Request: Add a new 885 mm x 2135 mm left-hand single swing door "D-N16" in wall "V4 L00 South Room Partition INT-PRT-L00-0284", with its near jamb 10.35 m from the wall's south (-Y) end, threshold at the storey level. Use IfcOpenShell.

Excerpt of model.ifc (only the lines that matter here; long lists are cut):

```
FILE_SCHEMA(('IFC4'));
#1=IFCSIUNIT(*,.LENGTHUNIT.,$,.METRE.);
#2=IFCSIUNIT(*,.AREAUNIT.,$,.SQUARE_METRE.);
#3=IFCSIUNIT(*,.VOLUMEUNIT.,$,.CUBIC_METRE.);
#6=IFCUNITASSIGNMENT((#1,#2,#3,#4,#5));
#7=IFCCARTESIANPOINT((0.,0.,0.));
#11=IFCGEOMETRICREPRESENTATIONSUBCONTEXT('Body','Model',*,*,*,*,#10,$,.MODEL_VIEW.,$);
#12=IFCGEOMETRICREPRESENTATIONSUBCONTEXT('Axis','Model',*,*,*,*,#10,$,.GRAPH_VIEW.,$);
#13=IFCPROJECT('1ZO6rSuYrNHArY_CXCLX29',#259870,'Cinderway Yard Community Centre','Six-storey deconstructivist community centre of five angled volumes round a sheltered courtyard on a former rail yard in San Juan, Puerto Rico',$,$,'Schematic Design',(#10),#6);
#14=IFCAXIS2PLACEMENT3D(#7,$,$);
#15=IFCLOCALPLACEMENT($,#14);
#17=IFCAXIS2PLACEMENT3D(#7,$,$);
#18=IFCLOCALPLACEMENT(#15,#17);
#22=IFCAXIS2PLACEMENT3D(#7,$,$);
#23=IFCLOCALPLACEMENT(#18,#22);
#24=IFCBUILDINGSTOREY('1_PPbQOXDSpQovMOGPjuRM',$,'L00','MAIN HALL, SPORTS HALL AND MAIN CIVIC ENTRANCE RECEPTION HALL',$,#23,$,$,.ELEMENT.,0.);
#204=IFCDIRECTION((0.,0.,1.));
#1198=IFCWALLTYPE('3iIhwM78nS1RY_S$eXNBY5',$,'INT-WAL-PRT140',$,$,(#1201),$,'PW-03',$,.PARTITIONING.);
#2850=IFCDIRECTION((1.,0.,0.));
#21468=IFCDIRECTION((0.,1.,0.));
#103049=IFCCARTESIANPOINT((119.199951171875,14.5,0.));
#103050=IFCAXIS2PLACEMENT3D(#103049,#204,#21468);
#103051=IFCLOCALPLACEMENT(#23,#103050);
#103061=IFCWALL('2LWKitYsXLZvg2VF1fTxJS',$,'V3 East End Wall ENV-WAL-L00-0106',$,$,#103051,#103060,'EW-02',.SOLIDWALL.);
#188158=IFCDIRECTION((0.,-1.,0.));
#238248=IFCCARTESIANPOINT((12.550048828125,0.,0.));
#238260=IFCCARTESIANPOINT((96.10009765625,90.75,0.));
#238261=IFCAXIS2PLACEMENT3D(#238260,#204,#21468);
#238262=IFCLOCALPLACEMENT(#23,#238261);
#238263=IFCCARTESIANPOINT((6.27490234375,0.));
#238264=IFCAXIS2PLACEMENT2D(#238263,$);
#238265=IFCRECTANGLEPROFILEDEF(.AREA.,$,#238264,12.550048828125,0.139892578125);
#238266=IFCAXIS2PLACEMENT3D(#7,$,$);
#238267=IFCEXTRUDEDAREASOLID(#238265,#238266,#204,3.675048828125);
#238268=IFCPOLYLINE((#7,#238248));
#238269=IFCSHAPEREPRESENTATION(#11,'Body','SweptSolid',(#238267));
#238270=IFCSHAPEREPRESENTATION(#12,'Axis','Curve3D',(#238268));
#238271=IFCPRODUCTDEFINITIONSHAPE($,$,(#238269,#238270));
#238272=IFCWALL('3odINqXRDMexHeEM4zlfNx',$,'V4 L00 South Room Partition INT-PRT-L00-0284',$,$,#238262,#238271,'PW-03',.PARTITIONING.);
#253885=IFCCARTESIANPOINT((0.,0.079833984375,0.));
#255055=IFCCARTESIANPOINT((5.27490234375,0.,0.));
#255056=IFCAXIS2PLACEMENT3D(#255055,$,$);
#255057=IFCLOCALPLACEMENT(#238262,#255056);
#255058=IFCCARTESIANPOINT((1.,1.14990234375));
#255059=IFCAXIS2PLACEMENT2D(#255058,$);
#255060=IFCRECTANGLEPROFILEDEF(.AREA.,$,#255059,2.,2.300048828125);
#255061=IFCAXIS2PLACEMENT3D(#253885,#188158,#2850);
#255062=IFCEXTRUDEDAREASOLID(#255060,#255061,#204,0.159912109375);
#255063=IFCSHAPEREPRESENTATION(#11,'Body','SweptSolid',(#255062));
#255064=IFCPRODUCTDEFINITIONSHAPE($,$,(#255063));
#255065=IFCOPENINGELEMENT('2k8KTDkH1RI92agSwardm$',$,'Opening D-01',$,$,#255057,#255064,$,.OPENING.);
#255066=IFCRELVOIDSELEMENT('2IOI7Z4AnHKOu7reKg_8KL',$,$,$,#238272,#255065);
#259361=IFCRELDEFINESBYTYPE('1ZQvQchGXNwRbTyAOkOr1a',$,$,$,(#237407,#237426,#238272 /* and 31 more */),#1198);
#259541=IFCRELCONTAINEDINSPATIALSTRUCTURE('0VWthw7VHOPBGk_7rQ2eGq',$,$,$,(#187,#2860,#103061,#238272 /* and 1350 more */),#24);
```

```python
import numpy as np
import ifcopenshell
import ifcopenshell.api.feature
import ifcopenshell.api.geometry
import ifcopenshell.api.root
import ifcopenshell.api.spatial
import ifcopenshell.geom
import ifcopenshell.util.element
import ifcopenshell.util.placement
import ifcopenshell.util.representation
import ifcopenshell.util.shape
import ifcopenshell.util.unit

model = ifcopenshell.open("model.ifc")
unit_scale = ifcopenshell.util.unit.calculate_unit_scale(model)
settings = ifcopenshell.geom.settings()


def volume(element):
    """Net volume in cubic metres, openings subtracted."""
    shape = ifcopenshell.geom.create_shape(settings, element)
    return ifcopenshell.util.shape.get_volume(shape.geometry)


wall = model.by_guid("3odINqXRDMexHeEM4zlfNx")
storey = ifcopenshell.util.element.get_container(wall, ifc_class="IfcBuildingStorey")
context = ifcopenshell.util.representation.get_context(model, "Model", "Body", "MODEL_VIEW")
before = volume(wall)

width, height, from_end, sill = 0.885, 2.135, 10.35, 0.0  # metres

# The wall runs along its own X axis, and the end named is its -X end.
wall_shape = ifcopenshell.geom.create_shape(settings, wall)
x, y, z = ifcopenshell.util.shape.get_vertices(wall_shape.geometry).T
start = x.min() + from_end
face, thickness = float(y.min()), float(y.max() - y.min())
wall_matrix = ifcopenshell.util.placement.get_local_placement(wall.ObjectPlacement)
level = ifcopenshell.util.placement.get_local_placement(storey.ObjectPlacement)[2, 3]


def in_wall(x, y):
    """Placement at x, y metres in the wall's axes, at sill height."""
    matrix = wall_matrix.copy()
    matrix[:, 3] = wall_matrix @ np.array([x / unit_scale, y / unit_scale, 0.0, 1.0])
    matrix[2, 3] = level + sill / unit_scale
    return matrix


# Opening: a box that overshoots both wall faces by 50 mm.
opening = ifcopenshell.api.root.create_entity(model, ifc_class="IfcOpeningElement", predefined_type="OPENING")
box = ifcopenshell.api.geometry.add_wall_representation(
    model, context=context, length=width, height=height, thickness=thickness + 0.1
)
ifcopenshell.api.geometry.assign_representation(model, product=opening, representation=box)
ifcopenshell.api.geometry.edit_object_placement(model, product=opening, matrix=in_wall(start, face - 0.05), is_si=False)
ifcopenshell.api.feature.add_feature(model, feature=opening, element=wall)

door = ifcopenshell.api.root.create_entity(model, ifc_class="IfcDoor", name="D-N16", predefined_type="DOOR")
door.OverallWidth, door.OverallHeight = width / unit_scale, height / unit_scale
door.OperationType = "SINGLE_SWING_LEFT"
body = ifcopenshell.api.geometry.add_door_representation(
    model,
    context=context,
    overall_width=door.OverallWidth,
    overall_height=door.OverallHeight,
    operation_type="SINGLE_SWING_LEFT",
    lining_properties={"LiningDepth": thickness / unit_scale, "ThresholdDepth": thickness / unit_scale},
)
ifcopenshell.api.geometry.assign_representation(model, product=door, representation=body)
ifcopenshell.api.spatial.assign_container(model, products=[door], relating_structure=storey)
ifcopenshell.api.feature.add_filling(model, opening=opening, element=door)

# The lining spans the wall, so the door starts at the wall face.
ifcopenshell.api.geometry.edit_object_placement(model, product=door, matrix=in_wall(start, face), is_si=False)

after = volume(wall)

print(f"wall volume {before:.3f} -> {after:.3f} m3")

model.write("model_edited.ifc")
```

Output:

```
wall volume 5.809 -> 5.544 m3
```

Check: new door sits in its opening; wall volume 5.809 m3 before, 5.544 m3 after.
